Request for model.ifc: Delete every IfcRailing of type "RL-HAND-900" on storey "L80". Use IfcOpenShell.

First a look at what the model holds.

```python
import ifcopenshell
import ifcopenshell.util.element

model = ifcopenshell.open("model.ifc")
print(model.schema)
storey = next(s for s in model.by_type("IfcBuildingStorey") if s.Name == "L80")
railings = [e for e in ifcopenshell.util.element.get_decomposition(storey) if e.is_a("IfcRailing")]
seen = {}
for e in railings:
    element_type = ifcopenshell.util.element.get_type(e)
    name = element_type.Name if element_type not in (None, e) else None
    seen[name] = seen.get(name, 0) + 1
for name, count in sorted(seen.items(), key=str):
    print(count, "x", name)
```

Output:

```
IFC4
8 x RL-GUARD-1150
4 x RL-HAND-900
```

```python
import ifcopenshell
import ifcopenshell.api.root
import ifcopenshell.util.element

model = ifcopenshell.open("model.ifc")

storey = next(s for s in model.by_type("IfcBuildingStorey") if s.Name == "L80")
railings = [e for e in ifcopenshell.util.element.get_decomposition(storey) if e.is_a("IfcRailing")]
targets = [e for e in railings if (t := ifcopenshell.util.element.get_type(e)) not in (None, e) and t.Name == "RL-HAND-900"]

for e in targets:
    ifcopenshell.api.root.remove_product(model, product=e)
print(len(targets), "removed")

model.write("model_edited.ifc")
```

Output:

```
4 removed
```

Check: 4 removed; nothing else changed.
